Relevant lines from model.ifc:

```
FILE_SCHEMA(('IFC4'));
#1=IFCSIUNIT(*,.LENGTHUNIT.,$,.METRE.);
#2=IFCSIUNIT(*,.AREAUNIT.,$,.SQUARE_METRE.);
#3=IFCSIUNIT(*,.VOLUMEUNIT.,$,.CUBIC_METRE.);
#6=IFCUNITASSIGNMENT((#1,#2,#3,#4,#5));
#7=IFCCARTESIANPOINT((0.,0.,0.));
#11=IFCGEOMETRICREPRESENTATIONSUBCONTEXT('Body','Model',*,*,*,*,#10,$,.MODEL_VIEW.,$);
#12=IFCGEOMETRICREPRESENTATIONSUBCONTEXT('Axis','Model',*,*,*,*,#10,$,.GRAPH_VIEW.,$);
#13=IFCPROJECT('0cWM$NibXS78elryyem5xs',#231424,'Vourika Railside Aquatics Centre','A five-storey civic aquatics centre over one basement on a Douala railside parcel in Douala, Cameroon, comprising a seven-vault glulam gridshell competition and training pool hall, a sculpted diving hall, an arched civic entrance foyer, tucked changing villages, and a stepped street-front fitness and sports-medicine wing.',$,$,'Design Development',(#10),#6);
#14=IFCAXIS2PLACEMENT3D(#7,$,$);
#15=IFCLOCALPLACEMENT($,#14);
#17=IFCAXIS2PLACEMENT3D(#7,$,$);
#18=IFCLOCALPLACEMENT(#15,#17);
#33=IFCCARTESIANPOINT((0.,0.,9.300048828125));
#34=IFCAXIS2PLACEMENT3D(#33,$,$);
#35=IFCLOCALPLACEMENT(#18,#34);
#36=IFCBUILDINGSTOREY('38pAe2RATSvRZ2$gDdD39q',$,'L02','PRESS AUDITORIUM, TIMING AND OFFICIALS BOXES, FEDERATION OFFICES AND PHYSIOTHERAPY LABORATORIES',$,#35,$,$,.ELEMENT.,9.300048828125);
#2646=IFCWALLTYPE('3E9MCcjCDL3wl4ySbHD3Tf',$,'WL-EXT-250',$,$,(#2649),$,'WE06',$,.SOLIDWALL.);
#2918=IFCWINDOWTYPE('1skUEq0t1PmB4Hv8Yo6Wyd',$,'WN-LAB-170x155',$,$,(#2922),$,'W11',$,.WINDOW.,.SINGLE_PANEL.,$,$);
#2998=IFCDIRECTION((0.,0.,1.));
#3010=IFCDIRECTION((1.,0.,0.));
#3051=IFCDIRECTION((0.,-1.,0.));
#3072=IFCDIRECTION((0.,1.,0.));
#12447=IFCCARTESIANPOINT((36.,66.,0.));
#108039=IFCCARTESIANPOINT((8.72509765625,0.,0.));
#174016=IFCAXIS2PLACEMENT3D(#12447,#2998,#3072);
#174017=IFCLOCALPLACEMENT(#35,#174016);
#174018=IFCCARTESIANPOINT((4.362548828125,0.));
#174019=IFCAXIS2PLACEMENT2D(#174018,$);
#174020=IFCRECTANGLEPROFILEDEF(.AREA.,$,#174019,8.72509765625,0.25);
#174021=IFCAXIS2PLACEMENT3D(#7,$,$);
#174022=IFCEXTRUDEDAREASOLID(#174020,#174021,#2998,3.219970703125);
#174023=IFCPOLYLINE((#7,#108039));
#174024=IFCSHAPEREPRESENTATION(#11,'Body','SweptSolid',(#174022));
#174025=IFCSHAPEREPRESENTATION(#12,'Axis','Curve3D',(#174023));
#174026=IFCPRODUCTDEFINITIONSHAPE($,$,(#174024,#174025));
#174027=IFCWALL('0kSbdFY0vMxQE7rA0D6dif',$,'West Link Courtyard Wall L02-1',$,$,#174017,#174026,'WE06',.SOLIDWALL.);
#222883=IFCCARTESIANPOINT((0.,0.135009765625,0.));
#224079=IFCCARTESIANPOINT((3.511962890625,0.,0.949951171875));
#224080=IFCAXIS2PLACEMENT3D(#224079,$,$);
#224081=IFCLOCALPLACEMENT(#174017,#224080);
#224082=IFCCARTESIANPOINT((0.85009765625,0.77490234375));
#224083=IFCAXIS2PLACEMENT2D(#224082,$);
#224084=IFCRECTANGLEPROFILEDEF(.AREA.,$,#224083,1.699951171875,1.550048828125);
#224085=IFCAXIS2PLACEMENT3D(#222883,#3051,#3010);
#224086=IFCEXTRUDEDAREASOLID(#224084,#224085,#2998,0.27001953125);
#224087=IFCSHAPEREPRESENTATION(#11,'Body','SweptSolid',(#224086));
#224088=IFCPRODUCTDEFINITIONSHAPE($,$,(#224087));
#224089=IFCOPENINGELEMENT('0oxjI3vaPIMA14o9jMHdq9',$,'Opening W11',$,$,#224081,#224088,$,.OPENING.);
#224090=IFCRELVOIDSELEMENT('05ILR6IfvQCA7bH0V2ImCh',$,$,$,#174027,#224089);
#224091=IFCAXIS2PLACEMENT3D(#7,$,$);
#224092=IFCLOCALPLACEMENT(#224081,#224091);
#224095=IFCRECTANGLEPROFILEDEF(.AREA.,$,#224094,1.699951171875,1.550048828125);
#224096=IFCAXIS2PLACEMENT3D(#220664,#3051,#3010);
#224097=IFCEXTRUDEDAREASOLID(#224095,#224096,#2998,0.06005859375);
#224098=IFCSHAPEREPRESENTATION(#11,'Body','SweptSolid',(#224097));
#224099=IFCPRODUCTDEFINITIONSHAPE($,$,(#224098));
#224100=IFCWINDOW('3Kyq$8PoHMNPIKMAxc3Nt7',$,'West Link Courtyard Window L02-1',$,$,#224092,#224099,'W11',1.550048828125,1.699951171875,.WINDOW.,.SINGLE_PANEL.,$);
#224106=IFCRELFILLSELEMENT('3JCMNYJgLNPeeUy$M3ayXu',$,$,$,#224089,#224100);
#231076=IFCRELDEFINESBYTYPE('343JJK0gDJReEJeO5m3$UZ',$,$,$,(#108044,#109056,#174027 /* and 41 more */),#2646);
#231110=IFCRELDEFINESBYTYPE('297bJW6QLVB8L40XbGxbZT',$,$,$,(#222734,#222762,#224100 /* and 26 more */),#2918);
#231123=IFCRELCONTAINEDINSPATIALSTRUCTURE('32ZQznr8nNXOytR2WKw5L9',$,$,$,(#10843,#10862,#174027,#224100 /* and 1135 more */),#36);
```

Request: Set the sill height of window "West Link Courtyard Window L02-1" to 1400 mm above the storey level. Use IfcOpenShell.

```python
import numpy as np
import ifcopenshell
import ifcopenshell.api.geometry
import ifcopenshell.geom
import ifcopenshell.util.element
import ifcopenshell.util.placement
import ifcopenshell.util.shape
import ifcopenshell.util.unit

model = ifcopenshell.open("model.ifc")
unit_scale = ifcopenshell.util.unit.calculate_unit_scale(model)

window = model.by_guid("3Kyq$8PoHMNPIKMAxc3Nt7")
opening = window.FillsVoids[0].RelatingOpeningElement
storey = ifcopenshell.util.element.get_container(window, ifc_class="IfcBuildingStorey")
level = ifcopenshell.util.placement.get_local_placement(storey.ObjectPlacement)[2, 3]

# The opening's origin need not be at the sill, so measure its lowest point.
shape = ifcopenshell.geom.create_shape(ifcopenshell.geom.settings(), opening)
bottom = ifcopenshell.util.shape.get_shape_bottom_elevation(shape, shape.geometry) / unit_scale
dz = level + 1.4 / unit_scale - bottom

shift = np.array([0.0, 0.0, dz])
# The window is placed relative to its opening, so it follows when the opening moves.
matrix = ifcopenshell.util.placement.get_local_placement(opening.ObjectPlacement)
matrix[:3, 3] += shift
ifcopenshell.api.geometry.edit_object_placement(
    model, product=opening, matrix=matrix, is_si=False, should_transform_children=True
)

print(f"moved by {dz * unit_scale:+.3f} m")

model.write("model_edited.ifc")
```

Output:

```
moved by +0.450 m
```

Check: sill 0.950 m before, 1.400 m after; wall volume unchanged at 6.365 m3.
